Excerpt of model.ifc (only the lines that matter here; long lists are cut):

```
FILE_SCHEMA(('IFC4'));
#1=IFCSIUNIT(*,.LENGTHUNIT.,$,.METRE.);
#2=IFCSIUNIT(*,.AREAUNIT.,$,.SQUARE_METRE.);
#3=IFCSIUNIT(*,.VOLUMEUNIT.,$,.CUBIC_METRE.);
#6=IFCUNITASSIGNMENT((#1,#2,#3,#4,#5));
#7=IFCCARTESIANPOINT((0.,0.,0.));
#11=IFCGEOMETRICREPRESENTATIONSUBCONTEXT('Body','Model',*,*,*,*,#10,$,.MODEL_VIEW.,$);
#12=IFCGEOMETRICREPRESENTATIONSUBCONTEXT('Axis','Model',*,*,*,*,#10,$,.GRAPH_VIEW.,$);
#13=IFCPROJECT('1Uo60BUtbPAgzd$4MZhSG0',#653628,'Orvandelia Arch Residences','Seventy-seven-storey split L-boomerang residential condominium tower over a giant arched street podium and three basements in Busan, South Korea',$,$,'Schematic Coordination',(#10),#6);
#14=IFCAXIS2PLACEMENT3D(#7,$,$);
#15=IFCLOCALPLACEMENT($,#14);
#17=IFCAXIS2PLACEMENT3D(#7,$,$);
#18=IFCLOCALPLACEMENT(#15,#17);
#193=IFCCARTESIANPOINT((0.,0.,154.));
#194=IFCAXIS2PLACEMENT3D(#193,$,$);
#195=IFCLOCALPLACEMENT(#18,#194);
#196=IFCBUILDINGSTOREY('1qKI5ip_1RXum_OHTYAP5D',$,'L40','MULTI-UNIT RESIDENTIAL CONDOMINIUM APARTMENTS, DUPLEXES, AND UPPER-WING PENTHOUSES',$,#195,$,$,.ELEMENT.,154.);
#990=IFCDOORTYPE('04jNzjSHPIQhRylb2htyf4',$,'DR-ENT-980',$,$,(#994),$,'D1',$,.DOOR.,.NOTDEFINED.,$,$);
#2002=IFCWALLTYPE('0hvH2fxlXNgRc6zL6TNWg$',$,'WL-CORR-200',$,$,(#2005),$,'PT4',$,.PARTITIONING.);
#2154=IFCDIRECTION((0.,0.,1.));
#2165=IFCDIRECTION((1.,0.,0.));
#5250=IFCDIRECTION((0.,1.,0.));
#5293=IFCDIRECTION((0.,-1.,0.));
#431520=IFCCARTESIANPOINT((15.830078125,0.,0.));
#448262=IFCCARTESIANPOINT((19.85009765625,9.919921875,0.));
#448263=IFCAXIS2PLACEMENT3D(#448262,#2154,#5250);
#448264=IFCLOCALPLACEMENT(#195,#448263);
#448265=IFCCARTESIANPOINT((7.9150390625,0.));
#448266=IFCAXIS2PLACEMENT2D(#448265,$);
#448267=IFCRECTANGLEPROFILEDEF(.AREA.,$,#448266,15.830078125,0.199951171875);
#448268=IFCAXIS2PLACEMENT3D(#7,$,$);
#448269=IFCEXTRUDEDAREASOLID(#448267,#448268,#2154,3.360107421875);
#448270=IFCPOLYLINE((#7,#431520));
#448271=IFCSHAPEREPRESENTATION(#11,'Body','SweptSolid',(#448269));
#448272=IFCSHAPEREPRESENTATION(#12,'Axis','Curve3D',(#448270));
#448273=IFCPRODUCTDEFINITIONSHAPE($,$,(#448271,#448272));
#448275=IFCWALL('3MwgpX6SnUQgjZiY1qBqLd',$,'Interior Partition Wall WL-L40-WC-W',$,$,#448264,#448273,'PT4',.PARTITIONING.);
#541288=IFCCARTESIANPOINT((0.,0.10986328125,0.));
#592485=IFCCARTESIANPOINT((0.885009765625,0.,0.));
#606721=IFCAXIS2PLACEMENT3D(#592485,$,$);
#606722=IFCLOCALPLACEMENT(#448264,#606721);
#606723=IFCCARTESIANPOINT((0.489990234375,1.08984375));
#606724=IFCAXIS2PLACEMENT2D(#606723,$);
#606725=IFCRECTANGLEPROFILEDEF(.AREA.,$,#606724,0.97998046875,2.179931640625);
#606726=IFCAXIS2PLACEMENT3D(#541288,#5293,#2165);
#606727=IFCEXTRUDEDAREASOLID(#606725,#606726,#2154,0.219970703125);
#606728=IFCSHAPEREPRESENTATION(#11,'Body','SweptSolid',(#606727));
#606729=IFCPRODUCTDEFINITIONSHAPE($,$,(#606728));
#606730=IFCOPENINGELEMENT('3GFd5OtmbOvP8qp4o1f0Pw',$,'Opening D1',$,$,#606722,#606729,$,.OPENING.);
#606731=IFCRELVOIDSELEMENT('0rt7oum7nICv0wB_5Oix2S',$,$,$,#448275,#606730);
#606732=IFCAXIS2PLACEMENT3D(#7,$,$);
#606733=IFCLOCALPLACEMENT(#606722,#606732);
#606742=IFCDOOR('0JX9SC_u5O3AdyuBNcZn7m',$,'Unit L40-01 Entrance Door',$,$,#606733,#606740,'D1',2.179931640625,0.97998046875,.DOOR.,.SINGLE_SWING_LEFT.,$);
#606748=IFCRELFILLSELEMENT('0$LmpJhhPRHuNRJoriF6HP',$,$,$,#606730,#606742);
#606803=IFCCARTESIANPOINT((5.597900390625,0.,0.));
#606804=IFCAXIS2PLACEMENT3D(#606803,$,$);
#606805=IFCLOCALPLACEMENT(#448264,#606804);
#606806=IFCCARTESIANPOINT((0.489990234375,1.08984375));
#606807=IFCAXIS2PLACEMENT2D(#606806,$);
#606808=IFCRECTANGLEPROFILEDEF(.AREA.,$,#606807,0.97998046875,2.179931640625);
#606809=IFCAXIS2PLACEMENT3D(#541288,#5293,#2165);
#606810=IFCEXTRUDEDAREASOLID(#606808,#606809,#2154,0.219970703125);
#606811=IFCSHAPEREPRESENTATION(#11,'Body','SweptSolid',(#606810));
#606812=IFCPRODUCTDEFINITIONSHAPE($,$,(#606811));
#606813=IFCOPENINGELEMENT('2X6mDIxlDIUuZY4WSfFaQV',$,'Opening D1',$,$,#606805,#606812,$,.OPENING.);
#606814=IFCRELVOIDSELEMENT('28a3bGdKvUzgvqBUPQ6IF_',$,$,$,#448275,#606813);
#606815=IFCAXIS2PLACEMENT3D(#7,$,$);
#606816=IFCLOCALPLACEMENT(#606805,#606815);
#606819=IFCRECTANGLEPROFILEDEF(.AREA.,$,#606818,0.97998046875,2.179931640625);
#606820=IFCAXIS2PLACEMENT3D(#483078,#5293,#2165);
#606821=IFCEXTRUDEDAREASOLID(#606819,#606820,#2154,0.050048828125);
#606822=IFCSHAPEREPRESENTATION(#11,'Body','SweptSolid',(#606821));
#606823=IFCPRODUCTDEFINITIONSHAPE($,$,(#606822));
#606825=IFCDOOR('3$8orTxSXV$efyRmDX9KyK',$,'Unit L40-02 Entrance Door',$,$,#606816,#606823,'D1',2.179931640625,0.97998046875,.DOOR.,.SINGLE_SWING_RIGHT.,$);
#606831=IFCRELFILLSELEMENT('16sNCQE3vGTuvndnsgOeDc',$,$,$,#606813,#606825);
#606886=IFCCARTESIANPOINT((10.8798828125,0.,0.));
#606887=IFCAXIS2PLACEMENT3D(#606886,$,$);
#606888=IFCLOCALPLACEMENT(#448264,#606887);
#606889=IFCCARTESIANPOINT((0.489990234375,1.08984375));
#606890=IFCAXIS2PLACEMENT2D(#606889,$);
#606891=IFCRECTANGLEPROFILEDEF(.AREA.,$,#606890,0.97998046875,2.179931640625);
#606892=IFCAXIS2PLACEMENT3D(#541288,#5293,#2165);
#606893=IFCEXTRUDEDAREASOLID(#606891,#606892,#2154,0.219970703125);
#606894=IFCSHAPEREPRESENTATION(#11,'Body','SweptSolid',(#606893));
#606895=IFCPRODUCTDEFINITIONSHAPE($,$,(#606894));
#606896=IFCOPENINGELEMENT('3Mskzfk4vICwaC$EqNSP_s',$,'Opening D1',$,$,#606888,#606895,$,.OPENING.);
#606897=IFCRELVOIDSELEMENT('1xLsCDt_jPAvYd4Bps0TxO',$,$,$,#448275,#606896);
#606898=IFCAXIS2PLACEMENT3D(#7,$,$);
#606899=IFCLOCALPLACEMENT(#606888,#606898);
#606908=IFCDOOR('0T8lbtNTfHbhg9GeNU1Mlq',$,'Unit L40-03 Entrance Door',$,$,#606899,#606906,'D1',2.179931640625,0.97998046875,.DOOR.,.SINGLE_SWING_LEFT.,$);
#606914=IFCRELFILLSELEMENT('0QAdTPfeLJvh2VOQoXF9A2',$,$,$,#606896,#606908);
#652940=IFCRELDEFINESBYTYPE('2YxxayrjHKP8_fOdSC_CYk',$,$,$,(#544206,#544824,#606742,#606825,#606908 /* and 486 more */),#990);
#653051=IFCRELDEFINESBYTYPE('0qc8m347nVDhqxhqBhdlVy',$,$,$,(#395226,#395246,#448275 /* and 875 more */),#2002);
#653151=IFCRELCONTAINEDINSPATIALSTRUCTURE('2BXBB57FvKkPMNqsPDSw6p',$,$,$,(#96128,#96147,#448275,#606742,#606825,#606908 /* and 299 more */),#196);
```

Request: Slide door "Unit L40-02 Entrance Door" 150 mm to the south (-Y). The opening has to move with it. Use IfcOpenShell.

```python
import ifcopenshell
import ifcopenshell.api.geometry
import ifcopenshell.util.placement
import ifcopenshell.util.unit

model = ifcopenshell.open("model.ifc")
unit_scale = ifcopenshell.util.unit.calculate_unit_scale(model)

door = model.by_guid("3$8orTxSXV$efyRmDX9KyK")
opening = door.FillsVoids[0].RelatingOpeningElement
wall = opening.VoidsElements[0].RelatingBuildingElement

wall_matrix = ifcopenshell.util.placement.get_local_placement(wall.ObjectPlacement)
shift = wall_matrix[:3, 0] * -0.15 / unit_scale
before = ifcopenshell.util.placement.get_local_placement(door.ObjectPlacement)[:3, 3].copy()

# The door is placed relative to its opening, so it follows when the opening moves.
matrix = ifcopenshell.util.placement.get_local_placement(opening.ObjectPlacement)
matrix[:3, 3] += shift
ifcopenshell.api.geometry.edit_object_placement(
    model, product=opening, matrix=matrix, is_si=False, should_transform_children=True
)

after = ifcopenshell.util.placement.get_local_placement(door.ObjectPlacement)[:3, 3]
print("door moved by", (after - before).round(3) + 0.0)

model.write("model_updated.ifc")
```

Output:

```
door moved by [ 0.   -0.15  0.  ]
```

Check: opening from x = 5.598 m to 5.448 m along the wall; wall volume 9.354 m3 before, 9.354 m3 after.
